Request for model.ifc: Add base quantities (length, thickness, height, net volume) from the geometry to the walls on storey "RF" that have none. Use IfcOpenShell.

First a look at what the model holds.

```python
import ifcopenshell
import ifcopenshell.util.element
import ifcopenshell.util.unit

model = ifcopenshell.open("model.ifc")
print(model.schema)
for unit_type in ("LENGTHUNIT", "AREAUNIT", "VOLUMEUNIT"):
    print(unit_type, ifcopenshell.util.unit.calculate_unit_scale(model, unit_type))
storey = next(s for s in model.by_type("IfcBuildingStorey") if s.Name == "RF")
walls = [e for e in ifcopenshell.util.element.get_decomposition(storey) if e.is_a("IfcWall")]
for e in sorted(walls, key=lambda e: e.id()):
    print(e.id(), e.is_a(), e.Name, list(ifcopenshell.util.element.get_psets(e, qtos_only=True)), sep=" | ")
```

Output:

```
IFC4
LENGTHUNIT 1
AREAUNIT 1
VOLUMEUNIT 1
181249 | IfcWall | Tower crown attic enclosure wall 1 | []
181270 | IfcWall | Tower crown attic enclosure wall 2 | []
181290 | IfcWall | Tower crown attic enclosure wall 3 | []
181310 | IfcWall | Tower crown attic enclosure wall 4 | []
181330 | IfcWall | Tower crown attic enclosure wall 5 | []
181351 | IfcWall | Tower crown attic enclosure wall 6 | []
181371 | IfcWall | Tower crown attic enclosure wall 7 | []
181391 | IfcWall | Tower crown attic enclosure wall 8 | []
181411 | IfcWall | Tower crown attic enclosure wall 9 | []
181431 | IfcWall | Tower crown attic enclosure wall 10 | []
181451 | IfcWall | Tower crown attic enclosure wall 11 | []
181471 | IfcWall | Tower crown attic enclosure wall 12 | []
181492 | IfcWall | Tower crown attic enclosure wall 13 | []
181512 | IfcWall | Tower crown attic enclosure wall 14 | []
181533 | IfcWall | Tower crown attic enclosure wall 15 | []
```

```python
import ifcopenshell
import ifcopenshell.api.pset
import ifcopenshell.geom
import ifcopenshell.util.element
import ifcopenshell.util.shape
import ifcopenshell.util.unit

model = ifcopenshell.open("model.ifc")
unit_scale = ifcopenshell.util.unit.calculate_unit_scale(model)
volume_scale = ifcopenshell.util.unit.calculate_unit_scale(model, "VOLUMEUNIT")
settings = ifcopenshell.geom.settings()

storey = next(s for s in model.by_type("IfcBuildingStorey") if s.Name == "RF")
walls = [e for e in ifcopenshell.util.element.get_decomposition(storey) if e.is_a("IfcWall")]

for e in sorted(walls, key=lambda e: e.id()):
    if ifcopenshell.util.element.get_psets(e, qtos_only=True, should_inherit=False):
        continue
    # Geometry comes back in metres, in the element's own axes.
    shape = ifcopenshell.geom.create_shape(settings, e)
    values = {
        "Length": ifcopenshell.util.shape.get_x(shape.geometry) / unit_scale,
        "Width": ifcopenshell.util.shape.get_y(shape.geometry) / unit_scale,
        "Height": ifcopenshell.util.shape.get_z(shape.geometry) / unit_scale,
        "NetVolume": ifcopenshell.util.shape.get_volume(shape.geometry) / volume_scale,
    }
    qto = ifcopenshell.api.pset.add_qto(model, product=e, name="Qto_WallBaseQuantities")
    ifcopenshell.api.pset.edit_qto(model, qto=qto, properties=values)
    print(e.id(), {k: round(v, 3) for k, v in values.items()})

model.write("model_edited.ifc")
```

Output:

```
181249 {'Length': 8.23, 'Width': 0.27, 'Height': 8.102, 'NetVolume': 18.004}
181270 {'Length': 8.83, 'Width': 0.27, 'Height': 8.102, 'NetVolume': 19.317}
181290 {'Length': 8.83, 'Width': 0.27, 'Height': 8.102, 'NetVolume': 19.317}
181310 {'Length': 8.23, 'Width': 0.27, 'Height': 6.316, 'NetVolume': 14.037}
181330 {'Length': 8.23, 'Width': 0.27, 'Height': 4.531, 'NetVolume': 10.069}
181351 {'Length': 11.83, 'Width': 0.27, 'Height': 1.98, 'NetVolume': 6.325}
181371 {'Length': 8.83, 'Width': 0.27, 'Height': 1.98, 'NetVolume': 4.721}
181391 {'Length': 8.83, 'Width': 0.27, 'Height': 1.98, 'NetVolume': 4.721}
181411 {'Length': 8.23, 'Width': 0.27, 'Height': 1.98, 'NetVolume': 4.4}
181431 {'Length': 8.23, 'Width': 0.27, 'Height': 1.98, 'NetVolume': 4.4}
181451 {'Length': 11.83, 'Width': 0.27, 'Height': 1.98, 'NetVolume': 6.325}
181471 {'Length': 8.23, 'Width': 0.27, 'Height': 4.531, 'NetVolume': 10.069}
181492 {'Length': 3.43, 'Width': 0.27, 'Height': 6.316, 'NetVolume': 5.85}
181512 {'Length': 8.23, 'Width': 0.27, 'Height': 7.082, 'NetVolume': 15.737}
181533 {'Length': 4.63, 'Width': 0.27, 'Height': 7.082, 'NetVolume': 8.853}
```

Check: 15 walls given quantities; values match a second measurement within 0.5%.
